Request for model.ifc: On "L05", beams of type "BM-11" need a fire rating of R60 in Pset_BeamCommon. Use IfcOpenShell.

First a look at what the model holds.

```python
import ifcopenshell
import ifcopenshell.util.element

model = ifcopenshell.open("model.ifc")
print(model.schema)
storey = next(s for s in model.by_type("IfcBuildingStorey") if s.Name == "L05")
beams = [e for e in ifcopenshell.util.element.get_decomposition(storey) if e.is_a("IfcBeam")]
seen = {}
for e in beams:
    element_type = ifcopenshell.util.element.get_type(e)
    key = (element_type.Name if element_type != e and element_type else None, ifcopenshell.util.element.get_pset(e, "Pset_BeamCommon", "FireRating"))
    seen[key] = seen.get(key, 0) + 1
for (name, value), count in sorted(seen.items(), key=str):
    print(count, "x", name, "|", value)
```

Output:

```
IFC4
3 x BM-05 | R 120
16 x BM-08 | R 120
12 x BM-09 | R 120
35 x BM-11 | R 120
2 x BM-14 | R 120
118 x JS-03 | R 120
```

```python
import ifcopenshell
import ifcopenshell.api.pset
import ifcopenshell.util.element

model = ifcopenshell.open("model.ifc")

storey = next(s for s in model.by_type("IfcBuildingStorey") if s.Name == "L05")
beams = [e for e in ifcopenshell.util.element.get_decomposition(storey) if e.is_a("IfcBeam")]

count = 0
for e in beams:
    element_type = ifcopenshell.util.element.get_type(e)
    if element_type in (None, e) or element_type.Name != "BM-11":
        continue
    # add_pset returns the element's existing set when there is one.
    pset = ifcopenshell.api.pset.add_pset(model, product=e, name="Pset_BeamCommon")
    ifcopenshell.api.pset.edit_pset(model, pset=pset, properties={"FireRating": "R60"})
    count += 1

print(count, "beams updated")

model.write("model_v2.ifc")
```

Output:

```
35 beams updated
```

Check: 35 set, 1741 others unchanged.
